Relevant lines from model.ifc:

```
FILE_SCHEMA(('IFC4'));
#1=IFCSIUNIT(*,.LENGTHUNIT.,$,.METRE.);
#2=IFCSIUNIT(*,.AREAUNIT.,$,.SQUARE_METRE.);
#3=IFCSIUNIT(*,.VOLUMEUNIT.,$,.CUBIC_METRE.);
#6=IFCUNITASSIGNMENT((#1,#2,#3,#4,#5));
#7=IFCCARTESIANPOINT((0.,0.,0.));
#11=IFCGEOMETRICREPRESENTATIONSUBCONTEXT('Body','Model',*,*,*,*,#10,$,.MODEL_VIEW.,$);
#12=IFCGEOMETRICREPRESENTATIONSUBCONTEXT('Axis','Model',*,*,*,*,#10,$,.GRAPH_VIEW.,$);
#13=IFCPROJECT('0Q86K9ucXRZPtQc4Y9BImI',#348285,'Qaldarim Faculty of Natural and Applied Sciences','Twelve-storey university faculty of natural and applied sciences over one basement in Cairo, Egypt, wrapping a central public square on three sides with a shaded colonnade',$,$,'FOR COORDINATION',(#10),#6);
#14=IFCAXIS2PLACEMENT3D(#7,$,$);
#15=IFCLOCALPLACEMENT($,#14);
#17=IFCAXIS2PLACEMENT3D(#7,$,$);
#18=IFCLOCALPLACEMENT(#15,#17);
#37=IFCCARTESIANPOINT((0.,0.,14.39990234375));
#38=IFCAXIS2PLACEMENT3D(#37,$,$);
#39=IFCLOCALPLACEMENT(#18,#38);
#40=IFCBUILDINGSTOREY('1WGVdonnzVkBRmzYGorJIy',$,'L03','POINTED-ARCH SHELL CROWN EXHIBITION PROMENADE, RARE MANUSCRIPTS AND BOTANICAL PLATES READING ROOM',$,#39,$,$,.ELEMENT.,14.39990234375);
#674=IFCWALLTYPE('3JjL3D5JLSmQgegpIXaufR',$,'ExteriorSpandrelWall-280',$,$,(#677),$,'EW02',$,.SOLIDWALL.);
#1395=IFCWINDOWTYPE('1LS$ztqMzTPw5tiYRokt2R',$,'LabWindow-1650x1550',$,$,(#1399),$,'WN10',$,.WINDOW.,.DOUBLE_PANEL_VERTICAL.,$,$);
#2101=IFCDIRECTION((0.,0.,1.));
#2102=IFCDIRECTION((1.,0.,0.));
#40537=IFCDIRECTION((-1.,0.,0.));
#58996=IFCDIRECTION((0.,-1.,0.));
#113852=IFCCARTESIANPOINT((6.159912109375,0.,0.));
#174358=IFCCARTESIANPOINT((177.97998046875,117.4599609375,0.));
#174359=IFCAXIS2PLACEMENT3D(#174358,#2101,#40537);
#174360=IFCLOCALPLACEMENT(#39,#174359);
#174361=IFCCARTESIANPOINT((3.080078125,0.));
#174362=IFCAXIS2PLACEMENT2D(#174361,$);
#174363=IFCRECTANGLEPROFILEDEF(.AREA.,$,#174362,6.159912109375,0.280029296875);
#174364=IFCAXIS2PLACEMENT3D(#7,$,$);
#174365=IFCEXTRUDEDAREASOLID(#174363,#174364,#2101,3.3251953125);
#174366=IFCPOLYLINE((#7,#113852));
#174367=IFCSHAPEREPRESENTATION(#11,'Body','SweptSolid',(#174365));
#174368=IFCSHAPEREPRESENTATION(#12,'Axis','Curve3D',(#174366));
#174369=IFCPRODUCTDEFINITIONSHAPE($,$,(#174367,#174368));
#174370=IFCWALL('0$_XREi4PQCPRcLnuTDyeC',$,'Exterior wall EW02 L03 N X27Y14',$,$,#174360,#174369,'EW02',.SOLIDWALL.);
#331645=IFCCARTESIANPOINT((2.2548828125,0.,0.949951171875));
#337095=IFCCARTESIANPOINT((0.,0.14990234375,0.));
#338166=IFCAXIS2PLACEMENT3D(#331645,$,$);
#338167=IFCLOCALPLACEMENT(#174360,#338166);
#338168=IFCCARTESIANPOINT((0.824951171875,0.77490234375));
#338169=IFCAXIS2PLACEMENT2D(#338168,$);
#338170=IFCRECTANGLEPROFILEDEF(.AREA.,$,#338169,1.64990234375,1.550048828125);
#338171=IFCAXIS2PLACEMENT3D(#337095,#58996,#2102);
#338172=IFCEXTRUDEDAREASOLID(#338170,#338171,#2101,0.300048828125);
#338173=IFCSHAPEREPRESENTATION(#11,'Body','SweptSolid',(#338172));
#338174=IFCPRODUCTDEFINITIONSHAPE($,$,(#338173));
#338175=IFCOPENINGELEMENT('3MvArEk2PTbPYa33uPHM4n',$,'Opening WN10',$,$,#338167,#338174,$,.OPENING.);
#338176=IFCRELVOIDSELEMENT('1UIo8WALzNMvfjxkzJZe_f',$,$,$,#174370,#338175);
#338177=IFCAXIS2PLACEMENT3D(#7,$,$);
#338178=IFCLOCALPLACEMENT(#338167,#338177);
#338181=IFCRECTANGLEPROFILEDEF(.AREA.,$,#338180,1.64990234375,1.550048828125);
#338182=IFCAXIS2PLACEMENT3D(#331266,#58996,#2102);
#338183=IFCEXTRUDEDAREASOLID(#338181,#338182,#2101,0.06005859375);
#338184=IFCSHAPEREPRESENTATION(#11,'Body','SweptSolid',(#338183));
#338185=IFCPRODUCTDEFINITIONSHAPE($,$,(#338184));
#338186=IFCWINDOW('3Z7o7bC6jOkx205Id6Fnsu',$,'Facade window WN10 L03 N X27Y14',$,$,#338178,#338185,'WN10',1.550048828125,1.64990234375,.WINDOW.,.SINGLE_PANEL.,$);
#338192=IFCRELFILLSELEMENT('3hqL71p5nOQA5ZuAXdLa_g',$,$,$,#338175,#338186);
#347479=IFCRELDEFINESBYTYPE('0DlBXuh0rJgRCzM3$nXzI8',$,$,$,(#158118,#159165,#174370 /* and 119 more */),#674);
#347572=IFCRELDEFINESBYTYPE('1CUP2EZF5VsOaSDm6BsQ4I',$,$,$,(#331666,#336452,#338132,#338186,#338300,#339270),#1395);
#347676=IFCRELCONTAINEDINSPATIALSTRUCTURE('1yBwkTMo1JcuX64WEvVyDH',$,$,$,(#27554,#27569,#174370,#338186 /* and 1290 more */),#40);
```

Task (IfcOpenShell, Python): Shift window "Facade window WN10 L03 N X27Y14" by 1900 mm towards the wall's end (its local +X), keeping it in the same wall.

```python
import ifcopenshell
import ifcopenshell.api.geometry
import ifcopenshell.util.placement
import ifcopenshell.util.unit

model = ifcopenshell.open("model.ifc")
unit_scale = ifcopenshell.util.unit.calculate_unit_scale(model)

window = model.by_guid("3Z7o7bC6jOkx205Id6Fnsu")
opening = window.FillsVoids[0].RelatingOpeningElement
wall = opening.VoidsElements[0].RelatingBuildingElement

wall_matrix = ifcopenshell.util.placement.get_local_placement(wall.ObjectPlacement)
shift = wall_matrix[:3, 0] * 1.9 / unit_scale
before = ifcopenshell.util.placement.get_local_placement(window.ObjectPlacement)[:3, 3].copy()

# The window is placed relative to its opening, so it follows when the opening moves.
matrix = ifcopenshell.util.placement.get_local_placement(opening.ObjectPlacement)
matrix[:3, 3] += shift
ifcopenshell.api.geometry.edit_object_placement(
    model, product=opening, matrix=matrix, is_si=False, should_transform_children=True
)

after = ifcopenshell.util.placement.get_local_placement(window.ObjectPlacement)[:3, 3]
print("window moved by", (after - before).round(3) + 0.0)

model.write("model-out.ifc")
```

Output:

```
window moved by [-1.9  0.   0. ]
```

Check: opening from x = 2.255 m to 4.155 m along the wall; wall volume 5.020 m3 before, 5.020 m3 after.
